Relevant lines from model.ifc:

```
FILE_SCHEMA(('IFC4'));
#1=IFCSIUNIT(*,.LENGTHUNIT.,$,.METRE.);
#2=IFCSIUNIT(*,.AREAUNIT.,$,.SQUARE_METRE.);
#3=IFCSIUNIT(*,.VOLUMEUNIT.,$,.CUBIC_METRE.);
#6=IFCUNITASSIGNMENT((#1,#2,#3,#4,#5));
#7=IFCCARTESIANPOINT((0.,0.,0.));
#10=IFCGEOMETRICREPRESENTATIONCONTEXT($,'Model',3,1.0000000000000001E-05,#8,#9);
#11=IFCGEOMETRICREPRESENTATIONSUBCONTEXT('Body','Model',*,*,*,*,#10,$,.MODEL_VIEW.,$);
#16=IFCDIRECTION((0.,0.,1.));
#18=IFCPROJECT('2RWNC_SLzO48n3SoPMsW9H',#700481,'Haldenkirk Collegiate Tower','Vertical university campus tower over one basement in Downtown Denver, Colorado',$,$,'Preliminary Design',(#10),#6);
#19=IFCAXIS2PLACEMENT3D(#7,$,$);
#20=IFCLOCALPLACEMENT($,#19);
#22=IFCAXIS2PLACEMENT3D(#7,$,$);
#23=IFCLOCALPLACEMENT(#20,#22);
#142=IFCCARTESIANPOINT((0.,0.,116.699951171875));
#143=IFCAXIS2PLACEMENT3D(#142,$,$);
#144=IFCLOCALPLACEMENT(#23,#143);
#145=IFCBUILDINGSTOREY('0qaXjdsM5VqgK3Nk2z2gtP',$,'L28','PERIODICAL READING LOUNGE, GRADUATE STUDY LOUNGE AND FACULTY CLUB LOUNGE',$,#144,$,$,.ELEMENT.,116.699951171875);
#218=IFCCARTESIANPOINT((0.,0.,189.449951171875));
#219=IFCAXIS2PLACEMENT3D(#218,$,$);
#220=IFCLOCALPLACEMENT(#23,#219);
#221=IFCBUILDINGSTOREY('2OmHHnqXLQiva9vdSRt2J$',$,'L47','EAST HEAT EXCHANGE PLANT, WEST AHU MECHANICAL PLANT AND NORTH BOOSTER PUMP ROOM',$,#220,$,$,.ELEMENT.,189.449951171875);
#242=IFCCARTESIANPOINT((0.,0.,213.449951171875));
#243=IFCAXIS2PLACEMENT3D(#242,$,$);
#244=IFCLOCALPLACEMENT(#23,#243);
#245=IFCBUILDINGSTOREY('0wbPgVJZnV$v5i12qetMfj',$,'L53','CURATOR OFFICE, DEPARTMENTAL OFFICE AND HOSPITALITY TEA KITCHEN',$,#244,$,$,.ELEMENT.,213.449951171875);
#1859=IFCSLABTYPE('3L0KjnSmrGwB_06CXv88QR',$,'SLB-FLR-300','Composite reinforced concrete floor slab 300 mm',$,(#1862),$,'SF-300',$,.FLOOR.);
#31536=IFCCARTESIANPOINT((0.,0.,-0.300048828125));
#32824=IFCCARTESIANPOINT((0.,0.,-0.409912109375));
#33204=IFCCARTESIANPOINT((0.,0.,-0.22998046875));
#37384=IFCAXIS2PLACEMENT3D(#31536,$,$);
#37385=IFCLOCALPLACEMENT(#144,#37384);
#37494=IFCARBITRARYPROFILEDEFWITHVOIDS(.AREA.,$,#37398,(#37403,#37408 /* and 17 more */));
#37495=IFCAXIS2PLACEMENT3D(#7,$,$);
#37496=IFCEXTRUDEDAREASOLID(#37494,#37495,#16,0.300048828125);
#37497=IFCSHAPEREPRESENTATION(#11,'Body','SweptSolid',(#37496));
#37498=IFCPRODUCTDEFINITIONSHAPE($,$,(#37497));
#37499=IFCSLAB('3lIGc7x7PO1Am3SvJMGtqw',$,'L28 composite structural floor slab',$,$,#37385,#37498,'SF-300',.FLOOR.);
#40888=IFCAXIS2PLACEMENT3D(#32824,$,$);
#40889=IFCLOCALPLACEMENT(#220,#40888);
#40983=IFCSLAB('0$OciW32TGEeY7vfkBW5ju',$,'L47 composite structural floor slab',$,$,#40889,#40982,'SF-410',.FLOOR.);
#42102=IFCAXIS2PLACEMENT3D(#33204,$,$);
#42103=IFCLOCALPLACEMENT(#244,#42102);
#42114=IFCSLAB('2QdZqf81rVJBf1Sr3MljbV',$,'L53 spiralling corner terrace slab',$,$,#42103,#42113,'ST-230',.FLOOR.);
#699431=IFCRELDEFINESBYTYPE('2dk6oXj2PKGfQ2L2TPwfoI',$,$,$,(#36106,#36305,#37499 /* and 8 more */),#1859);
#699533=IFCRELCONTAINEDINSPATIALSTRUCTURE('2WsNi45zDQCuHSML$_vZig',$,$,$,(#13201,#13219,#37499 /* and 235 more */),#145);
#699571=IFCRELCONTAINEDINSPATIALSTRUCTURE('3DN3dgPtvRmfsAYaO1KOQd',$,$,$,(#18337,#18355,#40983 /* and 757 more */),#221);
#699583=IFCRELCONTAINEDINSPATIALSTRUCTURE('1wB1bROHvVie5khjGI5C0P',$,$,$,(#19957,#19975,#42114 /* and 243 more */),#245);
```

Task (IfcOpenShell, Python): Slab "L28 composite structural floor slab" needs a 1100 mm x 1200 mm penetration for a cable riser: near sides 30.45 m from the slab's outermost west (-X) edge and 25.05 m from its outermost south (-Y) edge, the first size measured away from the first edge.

```python
import numpy as np
import ifcopenshell
import ifcopenshell.api.feature
import ifcopenshell.api.geometry
import ifcopenshell.api.root
import ifcopenshell.geom
import ifcopenshell.util.placement
import ifcopenshell.util.representation
import ifcopenshell.util.shape
import ifcopenshell.util.unit

model = ifcopenshell.open("model.ifc")
unit_scale = ifcopenshell.util.unit.calculate_unit_scale(model)
settings = ifcopenshell.geom.settings()


def volume(element):
    """Net volume in cubic metres, openings subtracted."""
    shape = ifcopenshell.geom.create_shape(settings, element)
    return ifcopenshell.util.shape.get_volume(shape.geometry)


slab = model.by_guid("3lIGc7x7PO1Am3SvJMGtqw")
before = volume(slab)

# Extent in the slab's own axes, in metres. The edges named are its -X and -Y sides.
slab_shape = ifcopenshell.geom.create_shape(settings, slab)
vertices = ifcopenshell.util.shape.get_vertices(slab_shape.geometry)
x_min, y_min, bottom = vertices.min(axis=0)
top = vertices[:, 2].max()

opening = ifcopenshell.api.root.create_entity(model, ifc_class="IfcOpeningElement", name="Cable riser opening", predefined_type="OPENING")
context = ifcopenshell.util.representation.get_context(model, "Model", "Body", "MODEL_VIEW")
width, depth = 1.1, 1.2
outline = [(0.0, 0.0), (width, 0.0), (width, depth), (0.0, depth), (0.0, 0.0)]
# Overshoot both faces by 50 mm so the cut is clean.
shape = ifcopenshell.api.geometry.add_slab_representation(
    model, context=context, depth=top - bottom + 0.1, polyline=outline
)
ifcopenshell.api.geometry.assign_representation(model, product=opening, representation=shape)

matrix = ifcopenshell.util.placement.get_local_placement(slab.ObjectPlacement)
matrix[:, 3] = matrix @ np.append(np.array([x_min + 30.45, y_min + 25.05, bottom - 0.05]) / unit_scale, 1.0)
ifcopenshell.api.geometry.edit_object_placement(model, product=opening, matrix=matrix, is_si=False)
ifcopenshell.api.feature.add_feature(model, feature=opening, element=slab)

after = volume(slab)

print(f"slab volume {before:.3f} -> {after:.3f} m3")

model.write("model_v2.ifc")
```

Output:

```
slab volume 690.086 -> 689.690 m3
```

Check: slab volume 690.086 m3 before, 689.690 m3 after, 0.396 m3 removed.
